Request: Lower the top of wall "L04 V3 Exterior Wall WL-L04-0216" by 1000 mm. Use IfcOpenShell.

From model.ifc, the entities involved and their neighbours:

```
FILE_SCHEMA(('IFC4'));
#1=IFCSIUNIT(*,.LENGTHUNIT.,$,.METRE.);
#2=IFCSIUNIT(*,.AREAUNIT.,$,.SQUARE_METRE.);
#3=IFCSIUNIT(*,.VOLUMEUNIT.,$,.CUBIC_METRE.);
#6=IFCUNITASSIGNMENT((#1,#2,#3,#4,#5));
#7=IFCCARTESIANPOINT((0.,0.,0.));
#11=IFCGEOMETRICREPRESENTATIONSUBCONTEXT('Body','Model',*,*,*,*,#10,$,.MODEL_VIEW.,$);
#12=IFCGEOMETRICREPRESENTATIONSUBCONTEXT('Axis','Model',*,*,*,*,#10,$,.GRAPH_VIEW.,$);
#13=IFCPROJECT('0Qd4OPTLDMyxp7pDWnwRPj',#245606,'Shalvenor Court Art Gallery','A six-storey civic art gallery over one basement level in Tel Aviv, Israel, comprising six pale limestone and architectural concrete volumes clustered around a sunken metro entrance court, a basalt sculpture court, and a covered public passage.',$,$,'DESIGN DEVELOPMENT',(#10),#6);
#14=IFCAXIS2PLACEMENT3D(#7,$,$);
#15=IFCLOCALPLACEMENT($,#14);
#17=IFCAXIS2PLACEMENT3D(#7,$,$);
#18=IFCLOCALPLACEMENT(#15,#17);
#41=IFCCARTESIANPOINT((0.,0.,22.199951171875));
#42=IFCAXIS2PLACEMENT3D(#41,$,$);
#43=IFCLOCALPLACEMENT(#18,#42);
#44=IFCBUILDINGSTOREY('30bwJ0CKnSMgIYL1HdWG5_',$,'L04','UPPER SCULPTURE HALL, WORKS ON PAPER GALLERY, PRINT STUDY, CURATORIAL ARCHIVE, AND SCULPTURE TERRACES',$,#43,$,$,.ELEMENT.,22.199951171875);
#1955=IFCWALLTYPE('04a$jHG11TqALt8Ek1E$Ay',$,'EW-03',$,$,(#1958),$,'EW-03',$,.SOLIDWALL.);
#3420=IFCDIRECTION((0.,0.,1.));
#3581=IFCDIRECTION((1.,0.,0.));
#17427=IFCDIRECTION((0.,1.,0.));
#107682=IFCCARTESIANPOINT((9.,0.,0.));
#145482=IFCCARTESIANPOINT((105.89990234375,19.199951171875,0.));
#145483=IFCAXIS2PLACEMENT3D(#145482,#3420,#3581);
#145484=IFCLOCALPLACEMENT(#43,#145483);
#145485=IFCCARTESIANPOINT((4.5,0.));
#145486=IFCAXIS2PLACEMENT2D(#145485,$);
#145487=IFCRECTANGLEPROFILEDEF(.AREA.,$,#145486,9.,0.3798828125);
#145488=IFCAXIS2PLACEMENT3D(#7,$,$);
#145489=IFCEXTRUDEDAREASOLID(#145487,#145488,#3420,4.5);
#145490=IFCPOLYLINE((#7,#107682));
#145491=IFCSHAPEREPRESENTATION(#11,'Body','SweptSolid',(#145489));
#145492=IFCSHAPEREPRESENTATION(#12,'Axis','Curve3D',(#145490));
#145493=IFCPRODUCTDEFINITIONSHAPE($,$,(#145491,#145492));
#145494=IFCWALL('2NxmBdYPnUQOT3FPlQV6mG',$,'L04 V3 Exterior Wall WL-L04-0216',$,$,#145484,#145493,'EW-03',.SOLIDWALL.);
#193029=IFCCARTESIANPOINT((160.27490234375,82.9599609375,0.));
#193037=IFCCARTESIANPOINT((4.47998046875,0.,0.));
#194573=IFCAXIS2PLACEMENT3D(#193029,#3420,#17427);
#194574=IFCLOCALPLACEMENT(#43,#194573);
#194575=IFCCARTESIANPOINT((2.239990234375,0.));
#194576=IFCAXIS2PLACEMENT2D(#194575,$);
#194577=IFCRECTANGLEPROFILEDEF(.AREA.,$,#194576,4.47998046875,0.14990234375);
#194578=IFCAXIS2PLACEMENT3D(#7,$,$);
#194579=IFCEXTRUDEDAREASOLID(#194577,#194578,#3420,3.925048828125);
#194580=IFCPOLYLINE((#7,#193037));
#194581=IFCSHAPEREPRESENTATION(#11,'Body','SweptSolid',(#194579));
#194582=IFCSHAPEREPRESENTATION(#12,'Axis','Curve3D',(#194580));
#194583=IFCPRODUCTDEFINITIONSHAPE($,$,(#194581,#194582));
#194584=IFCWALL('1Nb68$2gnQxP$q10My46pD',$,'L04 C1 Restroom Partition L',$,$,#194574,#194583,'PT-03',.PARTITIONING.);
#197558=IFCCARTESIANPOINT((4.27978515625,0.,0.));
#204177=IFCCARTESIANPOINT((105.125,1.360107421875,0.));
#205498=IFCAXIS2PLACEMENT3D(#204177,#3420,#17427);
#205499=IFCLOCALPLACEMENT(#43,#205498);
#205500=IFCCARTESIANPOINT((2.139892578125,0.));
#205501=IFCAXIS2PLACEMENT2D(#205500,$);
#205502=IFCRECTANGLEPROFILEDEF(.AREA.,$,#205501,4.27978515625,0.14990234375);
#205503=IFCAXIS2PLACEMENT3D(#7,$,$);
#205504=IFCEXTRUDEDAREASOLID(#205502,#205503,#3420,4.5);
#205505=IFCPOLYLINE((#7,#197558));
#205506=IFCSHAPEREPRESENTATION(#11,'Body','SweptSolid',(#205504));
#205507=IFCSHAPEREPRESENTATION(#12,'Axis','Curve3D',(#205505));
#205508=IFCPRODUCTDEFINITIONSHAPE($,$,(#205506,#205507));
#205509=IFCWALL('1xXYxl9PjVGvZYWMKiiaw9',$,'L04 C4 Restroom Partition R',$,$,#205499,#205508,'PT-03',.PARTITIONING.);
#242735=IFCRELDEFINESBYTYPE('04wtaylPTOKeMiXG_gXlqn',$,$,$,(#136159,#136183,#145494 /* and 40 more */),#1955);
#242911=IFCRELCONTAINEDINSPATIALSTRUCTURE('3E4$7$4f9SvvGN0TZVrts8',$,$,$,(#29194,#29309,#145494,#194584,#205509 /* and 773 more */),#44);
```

```python
import ifcopenshell
import ifcopenshell.geom
import ifcopenshell.util.representation
import ifcopenshell.util.shape
import ifcopenshell.util.unit

model = ifcopenshell.open("model.ifc")
unit_scale = ifcopenshell.util.unit.calculate_unit_scale(model)
settings = ifcopenshell.geom.settings()


def volume(element):
    """Net volume in cubic metres, openings subtracted."""
    shape = ifcopenshell.geom.create_shape(settings, element)
    return ifcopenshell.util.shape.get_volume(shape.geometry)


wall = model.by_guid("2NxmBdYPnUQOT3FPlQV6mG")
before = volume(wall)

body = ifcopenshell.util.representation.get_representation(wall, "Model", "Body")
solid = body.Items[0]
old_height = solid.Depth
solid.Depth -= 1 / unit_scale
after = volume(wall)

print(f"height {old_height:g} -> {solid.Depth:g}, volume {before:.3f} -> {after:.3f} m3")

model.write("model_rev.ifc")
```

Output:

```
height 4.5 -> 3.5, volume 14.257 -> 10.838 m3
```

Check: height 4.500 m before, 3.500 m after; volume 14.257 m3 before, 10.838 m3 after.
